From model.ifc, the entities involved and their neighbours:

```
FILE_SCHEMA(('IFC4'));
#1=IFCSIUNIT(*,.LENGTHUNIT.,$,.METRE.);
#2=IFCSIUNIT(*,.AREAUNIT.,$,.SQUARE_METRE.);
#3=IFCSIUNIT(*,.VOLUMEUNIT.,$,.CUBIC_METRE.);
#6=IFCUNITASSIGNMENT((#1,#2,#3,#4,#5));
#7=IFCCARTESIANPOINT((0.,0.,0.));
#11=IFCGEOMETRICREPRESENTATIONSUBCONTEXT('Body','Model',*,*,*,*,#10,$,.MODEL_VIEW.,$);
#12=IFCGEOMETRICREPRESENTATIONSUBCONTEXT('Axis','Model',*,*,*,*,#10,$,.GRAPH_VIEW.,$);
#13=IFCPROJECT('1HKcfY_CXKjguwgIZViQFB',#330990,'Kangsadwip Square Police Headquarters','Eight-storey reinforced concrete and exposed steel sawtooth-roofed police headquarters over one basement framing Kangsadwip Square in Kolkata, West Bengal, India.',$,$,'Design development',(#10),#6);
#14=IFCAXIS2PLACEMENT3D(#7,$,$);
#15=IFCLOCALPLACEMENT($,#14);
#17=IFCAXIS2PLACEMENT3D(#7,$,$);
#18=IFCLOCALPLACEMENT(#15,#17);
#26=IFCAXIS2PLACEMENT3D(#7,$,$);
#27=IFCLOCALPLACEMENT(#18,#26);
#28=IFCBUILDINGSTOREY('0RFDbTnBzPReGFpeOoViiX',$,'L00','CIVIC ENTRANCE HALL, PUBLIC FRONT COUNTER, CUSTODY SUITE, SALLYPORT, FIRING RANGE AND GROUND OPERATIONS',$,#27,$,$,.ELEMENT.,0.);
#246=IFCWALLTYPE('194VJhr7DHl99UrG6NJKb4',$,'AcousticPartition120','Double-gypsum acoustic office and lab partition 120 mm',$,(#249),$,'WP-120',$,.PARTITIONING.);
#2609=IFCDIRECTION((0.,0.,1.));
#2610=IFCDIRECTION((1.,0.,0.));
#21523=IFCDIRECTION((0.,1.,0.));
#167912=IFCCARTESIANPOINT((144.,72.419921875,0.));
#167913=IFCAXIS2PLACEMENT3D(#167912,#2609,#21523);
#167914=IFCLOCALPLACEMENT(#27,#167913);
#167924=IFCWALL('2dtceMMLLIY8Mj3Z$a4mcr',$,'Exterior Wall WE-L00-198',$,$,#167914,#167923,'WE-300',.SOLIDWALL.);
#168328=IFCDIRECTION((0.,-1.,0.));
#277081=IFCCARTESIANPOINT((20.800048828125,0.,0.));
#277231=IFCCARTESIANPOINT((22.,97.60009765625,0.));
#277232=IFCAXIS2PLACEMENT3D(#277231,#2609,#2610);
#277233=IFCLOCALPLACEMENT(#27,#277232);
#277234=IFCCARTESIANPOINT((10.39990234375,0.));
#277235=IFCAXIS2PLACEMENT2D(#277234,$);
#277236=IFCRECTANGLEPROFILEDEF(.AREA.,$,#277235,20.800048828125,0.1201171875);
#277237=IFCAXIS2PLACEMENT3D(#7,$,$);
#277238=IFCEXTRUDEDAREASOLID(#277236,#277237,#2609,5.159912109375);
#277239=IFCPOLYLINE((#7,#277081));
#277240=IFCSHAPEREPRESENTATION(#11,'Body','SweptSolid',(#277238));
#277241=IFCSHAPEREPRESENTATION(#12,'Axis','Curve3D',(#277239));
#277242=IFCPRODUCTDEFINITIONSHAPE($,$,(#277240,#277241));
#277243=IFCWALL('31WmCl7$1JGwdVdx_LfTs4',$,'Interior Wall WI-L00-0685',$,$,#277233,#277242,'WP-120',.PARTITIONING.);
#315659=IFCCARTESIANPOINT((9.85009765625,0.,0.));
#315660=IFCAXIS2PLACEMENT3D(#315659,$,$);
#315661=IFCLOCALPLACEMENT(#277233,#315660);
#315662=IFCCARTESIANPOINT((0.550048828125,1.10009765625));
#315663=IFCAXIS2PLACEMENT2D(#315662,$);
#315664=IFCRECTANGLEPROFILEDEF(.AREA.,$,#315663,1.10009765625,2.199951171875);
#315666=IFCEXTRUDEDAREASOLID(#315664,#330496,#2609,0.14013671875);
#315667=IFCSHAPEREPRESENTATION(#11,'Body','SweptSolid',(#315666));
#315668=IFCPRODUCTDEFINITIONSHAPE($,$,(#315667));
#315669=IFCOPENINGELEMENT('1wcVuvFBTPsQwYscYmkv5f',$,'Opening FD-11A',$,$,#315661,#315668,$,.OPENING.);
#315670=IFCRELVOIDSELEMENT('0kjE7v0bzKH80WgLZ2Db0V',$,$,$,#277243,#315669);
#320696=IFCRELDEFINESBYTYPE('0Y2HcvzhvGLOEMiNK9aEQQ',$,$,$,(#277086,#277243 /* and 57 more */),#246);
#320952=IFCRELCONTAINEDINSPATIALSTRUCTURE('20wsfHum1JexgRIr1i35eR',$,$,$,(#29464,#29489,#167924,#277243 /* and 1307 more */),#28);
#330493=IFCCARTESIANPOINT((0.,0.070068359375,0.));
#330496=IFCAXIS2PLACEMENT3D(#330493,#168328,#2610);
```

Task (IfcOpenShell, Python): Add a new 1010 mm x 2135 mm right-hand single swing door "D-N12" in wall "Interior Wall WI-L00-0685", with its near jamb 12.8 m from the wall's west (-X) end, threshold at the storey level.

```python
import numpy as np
import ifcopenshell
import ifcopenshell.api.feature
import ifcopenshell.api.geometry
import ifcopenshell.api.root
import ifcopenshell.api.spatial
import ifcopenshell.geom
import ifcopenshell.util.element
import ifcopenshell.util.placement
import ifcopenshell.util.representation
import ifcopenshell.util.shape
import ifcopenshell.util.unit

model = ifcopenshell.open("model.ifc")
unit_scale = ifcopenshell.util.unit.calculate_unit_scale(model)
settings = ifcopenshell.geom.settings()


def volume(element):
    """Net volume in cubic metres, openings subtracted."""
    shape = ifcopenshell.geom.create_shape(settings, element)
    return ifcopenshell.util.shape.get_volume(shape.geometry)


wall = model.by_guid("31WmCl7$1JGwdVdx_LfTs4")
storey = ifcopenshell.util.element.get_container(wall, ifc_class="IfcBuildingStorey")
context = ifcopenshell.util.representation.get_context(model, "Model", "Body", "MODEL_VIEW")
before = volume(wall)

width, height, from_end, sill = 1.01, 2.135, 12.8, 0.0  # metres

# The wall runs along its own X axis, and the end named is its -X end.
wall_shape = ifcopenshell.geom.create_shape(settings, wall)
x, y, z = ifcopenshell.util.shape.get_vertices(wall_shape.geometry).T
start = x.min() + from_end
face, thickness = float(y.min()), float(y.max() - y.min())
wall_matrix = ifcopenshell.util.placement.get_local_placement(wall.ObjectPlacement)
level = ifcopenshell.util.placement.get_local_placement(storey.ObjectPlacement)[2, 3]


def in_wall(x, y):
    """Placement at x, y metres in the wall's axes, at sill height."""
    matrix = wall_matrix.copy()
    matrix[:, 3] = wall_matrix @ np.array([x / unit_scale, y / unit_scale, 0.0, 1.0])
    matrix[2, 3] = level + sill / unit_scale
    return matrix


# Opening: a box that overshoots both wall faces by 50 mm.
opening = ifcopenshell.api.root.create_entity(model, ifc_class="IfcOpeningElement", predefined_type="OPENING")
box = ifcopenshell.api.geometry.add_wall_representation(
    model, context=context, length=width, height=height, thickness=thickness + 0.1
)
ifcopenshell.api.geometry.assign_representation(model, product=opening, representation=box)
ifcopenshell.api.geometry.edit_object_placement(model, product=opening, matrix=in_wall(start, face - 0.05), is_si=False)
ifcopenshell.api.feature.add_feature(model, feature=opening, element=wall)

door = ifcopenshell.api.root.create_entity(model, ifc_class="IfcDoor", name="D-N12", predefined_type="DOOR")
door.OverallWidth, door.OverallHeight = width / unit_scale, height / unit_scale
door.OperationType = "SINGLE_SWING_RIGHT"
body = ifcopenshell.api.geometry.add_door_representation(
    model,
    context=context,
    overall_width=door.OverallWidth,
    overall_height=door.OverallHeight,
    operation_type="SINGLE_SWING_RIGHT",
    lining_properties={"LiningDepth": thickness / unit_scale, "ThresholdDepth": thickness / unit_scale},
)
ifcopenshell.api.geometry.assign_representation(model, product=door, representation=body)
ifcopenshell.api.spatial.assign_container(model, products=[door], relating_structure=storey)
ifcopenshell.api.feature.add_filling(model, opening=opening, element=door)

# The lining spans the wall, so the door starts at the wall face.
ifcopenshell.api.geometry.edit_object_placement(model, product=door, matrix=in_wall(start, face), is_si=False)

after = volume(wall)

print(f"wall volume {before:.3f} -> {after:.3f} m3")

model.write("model_rev.ifc")
```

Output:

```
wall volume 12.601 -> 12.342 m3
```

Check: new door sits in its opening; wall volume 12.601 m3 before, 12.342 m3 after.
